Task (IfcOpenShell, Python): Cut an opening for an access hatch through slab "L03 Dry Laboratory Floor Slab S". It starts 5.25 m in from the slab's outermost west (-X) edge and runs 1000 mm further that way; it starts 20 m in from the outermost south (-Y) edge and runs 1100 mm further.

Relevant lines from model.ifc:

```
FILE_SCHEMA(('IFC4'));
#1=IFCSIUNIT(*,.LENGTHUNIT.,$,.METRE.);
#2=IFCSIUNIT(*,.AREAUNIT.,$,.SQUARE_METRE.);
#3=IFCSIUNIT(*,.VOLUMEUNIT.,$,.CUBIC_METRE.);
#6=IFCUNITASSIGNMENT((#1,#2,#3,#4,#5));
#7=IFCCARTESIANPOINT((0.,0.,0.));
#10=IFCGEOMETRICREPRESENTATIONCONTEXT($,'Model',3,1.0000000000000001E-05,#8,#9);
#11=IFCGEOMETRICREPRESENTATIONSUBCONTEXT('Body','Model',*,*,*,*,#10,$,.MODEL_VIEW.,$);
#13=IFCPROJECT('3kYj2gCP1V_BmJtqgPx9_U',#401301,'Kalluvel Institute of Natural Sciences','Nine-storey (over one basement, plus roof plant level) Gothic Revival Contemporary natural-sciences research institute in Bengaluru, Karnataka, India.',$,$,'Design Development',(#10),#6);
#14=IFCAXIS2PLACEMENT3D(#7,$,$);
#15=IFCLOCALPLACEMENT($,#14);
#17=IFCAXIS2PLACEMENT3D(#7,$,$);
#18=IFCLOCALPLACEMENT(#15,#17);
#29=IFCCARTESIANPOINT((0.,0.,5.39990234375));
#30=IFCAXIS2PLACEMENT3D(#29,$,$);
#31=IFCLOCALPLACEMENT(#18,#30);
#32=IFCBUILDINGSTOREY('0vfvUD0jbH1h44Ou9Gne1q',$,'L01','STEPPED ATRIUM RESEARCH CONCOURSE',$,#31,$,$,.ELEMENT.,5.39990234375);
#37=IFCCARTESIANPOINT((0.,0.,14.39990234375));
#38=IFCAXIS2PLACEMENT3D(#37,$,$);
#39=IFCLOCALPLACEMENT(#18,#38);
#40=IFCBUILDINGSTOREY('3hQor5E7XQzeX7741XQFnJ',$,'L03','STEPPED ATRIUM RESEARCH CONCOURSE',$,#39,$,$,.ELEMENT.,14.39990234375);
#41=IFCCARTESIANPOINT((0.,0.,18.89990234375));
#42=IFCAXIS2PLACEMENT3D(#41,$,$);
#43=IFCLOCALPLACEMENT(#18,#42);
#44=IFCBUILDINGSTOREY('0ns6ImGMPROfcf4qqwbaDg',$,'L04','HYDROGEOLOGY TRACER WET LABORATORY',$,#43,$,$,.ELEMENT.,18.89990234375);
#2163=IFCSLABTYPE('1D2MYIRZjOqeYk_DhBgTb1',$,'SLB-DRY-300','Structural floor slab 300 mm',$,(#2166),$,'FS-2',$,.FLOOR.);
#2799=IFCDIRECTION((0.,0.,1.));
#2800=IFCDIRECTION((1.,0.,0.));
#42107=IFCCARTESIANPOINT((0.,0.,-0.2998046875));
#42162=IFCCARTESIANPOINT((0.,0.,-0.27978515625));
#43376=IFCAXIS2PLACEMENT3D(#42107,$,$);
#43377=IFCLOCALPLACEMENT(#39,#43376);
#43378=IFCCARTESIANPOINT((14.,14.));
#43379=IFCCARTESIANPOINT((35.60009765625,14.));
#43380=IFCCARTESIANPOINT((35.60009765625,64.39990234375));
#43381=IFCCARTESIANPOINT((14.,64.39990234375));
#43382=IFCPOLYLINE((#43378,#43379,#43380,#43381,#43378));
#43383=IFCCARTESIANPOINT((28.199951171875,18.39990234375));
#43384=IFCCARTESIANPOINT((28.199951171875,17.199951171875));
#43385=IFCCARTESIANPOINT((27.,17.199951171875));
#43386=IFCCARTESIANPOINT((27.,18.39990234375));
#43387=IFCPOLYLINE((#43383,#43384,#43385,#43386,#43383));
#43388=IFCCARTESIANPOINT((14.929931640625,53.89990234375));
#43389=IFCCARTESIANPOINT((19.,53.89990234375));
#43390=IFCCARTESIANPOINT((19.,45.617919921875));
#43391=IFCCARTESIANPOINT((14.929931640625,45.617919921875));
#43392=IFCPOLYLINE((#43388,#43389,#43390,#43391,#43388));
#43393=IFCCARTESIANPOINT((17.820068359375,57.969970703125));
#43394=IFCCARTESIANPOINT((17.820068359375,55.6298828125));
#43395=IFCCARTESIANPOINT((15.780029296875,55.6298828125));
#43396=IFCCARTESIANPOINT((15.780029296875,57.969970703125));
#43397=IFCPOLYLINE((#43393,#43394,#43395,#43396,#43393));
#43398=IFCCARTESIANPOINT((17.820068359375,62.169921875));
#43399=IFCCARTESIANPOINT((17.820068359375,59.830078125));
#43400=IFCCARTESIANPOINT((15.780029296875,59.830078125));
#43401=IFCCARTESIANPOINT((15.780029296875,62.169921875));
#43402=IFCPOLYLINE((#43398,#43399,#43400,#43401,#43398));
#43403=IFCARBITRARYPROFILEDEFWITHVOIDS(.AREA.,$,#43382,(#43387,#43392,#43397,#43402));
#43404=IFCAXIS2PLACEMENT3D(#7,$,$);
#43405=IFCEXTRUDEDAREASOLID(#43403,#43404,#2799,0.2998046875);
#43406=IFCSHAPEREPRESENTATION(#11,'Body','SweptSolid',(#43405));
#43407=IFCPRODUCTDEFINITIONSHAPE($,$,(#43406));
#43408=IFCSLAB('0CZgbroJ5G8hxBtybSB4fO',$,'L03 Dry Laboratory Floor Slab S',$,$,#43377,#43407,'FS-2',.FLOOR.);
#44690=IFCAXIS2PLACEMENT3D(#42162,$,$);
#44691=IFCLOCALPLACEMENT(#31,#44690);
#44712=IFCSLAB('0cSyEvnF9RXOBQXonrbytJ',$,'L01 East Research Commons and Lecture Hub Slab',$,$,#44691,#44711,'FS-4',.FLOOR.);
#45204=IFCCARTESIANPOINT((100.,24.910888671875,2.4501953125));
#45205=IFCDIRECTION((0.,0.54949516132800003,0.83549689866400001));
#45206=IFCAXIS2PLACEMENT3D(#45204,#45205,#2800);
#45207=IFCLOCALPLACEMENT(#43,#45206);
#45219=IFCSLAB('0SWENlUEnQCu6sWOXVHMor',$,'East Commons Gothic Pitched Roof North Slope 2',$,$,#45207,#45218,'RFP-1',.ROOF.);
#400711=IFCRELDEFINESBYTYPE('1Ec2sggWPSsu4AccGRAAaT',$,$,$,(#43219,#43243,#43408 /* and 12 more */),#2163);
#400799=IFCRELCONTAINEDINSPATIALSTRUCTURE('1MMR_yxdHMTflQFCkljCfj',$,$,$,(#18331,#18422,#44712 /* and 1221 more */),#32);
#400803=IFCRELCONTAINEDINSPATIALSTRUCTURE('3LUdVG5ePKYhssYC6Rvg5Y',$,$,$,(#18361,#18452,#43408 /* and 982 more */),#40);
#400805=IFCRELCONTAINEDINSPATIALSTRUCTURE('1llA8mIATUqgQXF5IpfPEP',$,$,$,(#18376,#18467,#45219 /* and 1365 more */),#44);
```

```python
import numpy as np
import ifcopenshell
import ifcopenshell.api.feature
import ifcopenshell.api.geometry
import ifcopenshell.api.root
import ifcopenshell.geom
import ifcopenshell.util.placement
import ifcopenshell.util.representation
import ifcopenshell.util.shape
import ifcopenshell.util.unit

model = ifcopenshell.open("model.ifc")
unit_scale = ifcopenshell.util.unit.calculate_unit_scale(model)
settings = ifcopenshell.geom.settings()


def volume(element):
    """Net volume in cubic metres, openings subtracted."""
    shape = ifcopenshell.geom.create_shape(settings, element)
    return ifcopenshell.util.shape.get_volume(shape.geometry)


slab = model.by_guid("0CZgbroJ5G8hxBtybSB4fO")
before = volume(slab)

# Extent in the slab's own axes, in metres. The edges named are its -X and -Y sides.
slab_shape = ifcopenshell.geom.create_shape(settings, slab)
vertices = ifcopenshell.util.shape.get_vertices(slab_shape.geometry)
x_min, y_min, bottom = vertices.min(axis=0)
top = vertices[:, 2].max()

opening = ifcopenshell.api.root.create_entity(model, ifc_class="IfcOpeningElement", name="Access hatch opening", predefined_type="OPENING")
context = ifcopenshell.util.representation.get_context(model, "Model", "Body", "MODEL_VIEW")
width, depth = 1, 1.1
outline = [(0.0, 0.0), (width, 0.0), (width, depth), (0.0, depth), (0.0, 0.0)]
# Overshoot both faces by 50 mm so the cut is clean.
shape = ifcopenshell.api.geometry.add_slab_representation(
    model, context=context, depth=top - bottom + 0.1, polyline=outline
)
ifcopenshell.api.geometry.assign_representation(model, product=opening, representation=shape)

matrix = ifcopenshell.util.placement.get_local_placement(slab.ObjectPlacement)
matrix[:, 3] = matrix @ np.append(np.array([x_min + 5.25, y_min + 20, bottom - 0.05]) / unit_scale, 1.0)
ifcopenshell.api.geometry.edit_object_placement(model, product=opening, matrix=matrix, is_si=False)
ifcopenshell.api.feature.add_feature(model, feature=opening, element=slab)

after = volume(slab)

print(f"slab volume {before:.3f} -> {after:.3f} m3")

model.write("model_rev.ifc")
```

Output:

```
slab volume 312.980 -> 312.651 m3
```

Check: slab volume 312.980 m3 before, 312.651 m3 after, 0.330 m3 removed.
